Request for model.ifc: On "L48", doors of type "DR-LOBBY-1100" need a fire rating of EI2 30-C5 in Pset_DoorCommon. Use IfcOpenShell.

First a look at what the model holds.

```python
import ifcopenshell
import ifcopenshell.util.element

model = ifcopenshell.open("model.ifc")
print(model.schema)
storey = next(s for s in model.by_type("IfcBuildingStorey") if s.Name == "L48")
doors = [e for e in ifcopenshell.util.element.get_decomposition(storey) if e.is_a("IfcDoor")]
seen = {}
for e in doors:
    element_type = ifcopenshell.util.element.get_type(e)
    key = (element_type.Name if element_type != e and element_type else None, ifcopenshell.util.element.get_pset(e, "Pset_DoorCommon", "FireRating"))
    seen[key] = seen.get(key, 0) + 1
for (name, value), count in sorted(seen.items(), key=str):
    print(count, "x", name, "|", value)
```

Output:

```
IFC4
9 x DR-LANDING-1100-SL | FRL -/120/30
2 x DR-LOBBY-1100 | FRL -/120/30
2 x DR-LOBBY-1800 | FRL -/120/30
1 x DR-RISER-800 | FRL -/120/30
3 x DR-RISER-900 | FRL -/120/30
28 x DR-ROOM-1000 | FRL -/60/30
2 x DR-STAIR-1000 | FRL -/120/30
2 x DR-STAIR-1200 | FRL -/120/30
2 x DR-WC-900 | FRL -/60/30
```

```python
import ifcopenshell
import ifcopenshell.api.pset
import ifcopenshell.util.element

model = ifcopenshell.open("model.ifc")

storey = next(s for s in model.by_type("IfcBuildingStorey") if s.Name == "L48")
doors = [e for e in ifcopenshell.util.element.get_decomposition(storey) if e.is_a("IfcDoor")]

count = 0
for e in doors:
    element_type = ifcopenshell.util.element.get_type(e)
    if element_type in (None, e) or element_type.Name != "DR-LOBBY-1100":
        continue
    # add_pset returns the element's existing set when there is one.
    pset = ifcopenshell.api.pset.add_pset(model, product=e, name="Pset_DoorCommon")
    ifcopenshell.api.pset.edit_pset(model, pset=pset, properties={"FireRating": "EI2 30-C5"})
    count += 1

print(count, "doors updated")

model.write("model_rev.ifc")
```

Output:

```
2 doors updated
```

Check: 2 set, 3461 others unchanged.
